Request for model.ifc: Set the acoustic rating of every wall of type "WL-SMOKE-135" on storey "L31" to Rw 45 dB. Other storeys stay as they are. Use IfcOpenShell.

First a look at what the model holds.

```python
import ifcopenshell
import ifcopenshell.util.element

model = ifcopenshell.open("model.ifc")
print(model.schema)
storey = next(s for s in model.by_type("IfcBuildingStorey") if s.Name == "L31")
walls = [e for e in ifcopenshell.util.element.get_decomposition(storey) if e.is_a("IfcWall")]
seen = {}
for e in walls:
    element_type = ifcopenshell.util.element.get_type(e)
    key = (element_type.Name if element_type != e and element_type else None, ifcopenshell.util.element.get_pset(e, "Pset_WallCommon", "AcousticRating"))
    seen[key] = seen.get(key, 0) + 1
for (name, value), count in sorted(seen.items(), key=str):
    print(count, "x", name, "|", value)
```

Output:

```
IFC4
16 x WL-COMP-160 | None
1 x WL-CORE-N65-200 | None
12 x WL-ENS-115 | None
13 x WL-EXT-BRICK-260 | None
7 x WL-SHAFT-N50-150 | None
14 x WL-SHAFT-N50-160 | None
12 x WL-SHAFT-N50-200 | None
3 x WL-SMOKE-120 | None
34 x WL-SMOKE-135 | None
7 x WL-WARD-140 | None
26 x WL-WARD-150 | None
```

```python
import ifcopenshell
import ifcopenshell.api.pset
import ifcopenshell.util.element

model = ifcopenshell.open("model.ifc")

storey = next(s for s in model.by_type("IfcBuildingStorey") if s.Name == "L31")
walls = [e for e in ifcopenshell.util.element.get_decomposition(storey) if e.is_a("IfcWall")]

count = 0
for e in walls:
    element_type = ifcopenshell.util.element.get_type(e)
    if element_type in (None, e) or element_type.Name != "WL-SMOKE-135":
        continue
    # add_pset returns the element's existing set when there is one.
    pset = ifcopenshell.api.pset.add_pset(model, product=e, name="Pset_WallCommon")
    ifcopenshell.api.pset.edit_pset(model, pset=pset, properties={"AcousticRating": "Rw 45 dB"})
    count += 1

print(count, "walls updated")

model.write("model-out.ifc")
```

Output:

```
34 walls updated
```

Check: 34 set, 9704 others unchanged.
